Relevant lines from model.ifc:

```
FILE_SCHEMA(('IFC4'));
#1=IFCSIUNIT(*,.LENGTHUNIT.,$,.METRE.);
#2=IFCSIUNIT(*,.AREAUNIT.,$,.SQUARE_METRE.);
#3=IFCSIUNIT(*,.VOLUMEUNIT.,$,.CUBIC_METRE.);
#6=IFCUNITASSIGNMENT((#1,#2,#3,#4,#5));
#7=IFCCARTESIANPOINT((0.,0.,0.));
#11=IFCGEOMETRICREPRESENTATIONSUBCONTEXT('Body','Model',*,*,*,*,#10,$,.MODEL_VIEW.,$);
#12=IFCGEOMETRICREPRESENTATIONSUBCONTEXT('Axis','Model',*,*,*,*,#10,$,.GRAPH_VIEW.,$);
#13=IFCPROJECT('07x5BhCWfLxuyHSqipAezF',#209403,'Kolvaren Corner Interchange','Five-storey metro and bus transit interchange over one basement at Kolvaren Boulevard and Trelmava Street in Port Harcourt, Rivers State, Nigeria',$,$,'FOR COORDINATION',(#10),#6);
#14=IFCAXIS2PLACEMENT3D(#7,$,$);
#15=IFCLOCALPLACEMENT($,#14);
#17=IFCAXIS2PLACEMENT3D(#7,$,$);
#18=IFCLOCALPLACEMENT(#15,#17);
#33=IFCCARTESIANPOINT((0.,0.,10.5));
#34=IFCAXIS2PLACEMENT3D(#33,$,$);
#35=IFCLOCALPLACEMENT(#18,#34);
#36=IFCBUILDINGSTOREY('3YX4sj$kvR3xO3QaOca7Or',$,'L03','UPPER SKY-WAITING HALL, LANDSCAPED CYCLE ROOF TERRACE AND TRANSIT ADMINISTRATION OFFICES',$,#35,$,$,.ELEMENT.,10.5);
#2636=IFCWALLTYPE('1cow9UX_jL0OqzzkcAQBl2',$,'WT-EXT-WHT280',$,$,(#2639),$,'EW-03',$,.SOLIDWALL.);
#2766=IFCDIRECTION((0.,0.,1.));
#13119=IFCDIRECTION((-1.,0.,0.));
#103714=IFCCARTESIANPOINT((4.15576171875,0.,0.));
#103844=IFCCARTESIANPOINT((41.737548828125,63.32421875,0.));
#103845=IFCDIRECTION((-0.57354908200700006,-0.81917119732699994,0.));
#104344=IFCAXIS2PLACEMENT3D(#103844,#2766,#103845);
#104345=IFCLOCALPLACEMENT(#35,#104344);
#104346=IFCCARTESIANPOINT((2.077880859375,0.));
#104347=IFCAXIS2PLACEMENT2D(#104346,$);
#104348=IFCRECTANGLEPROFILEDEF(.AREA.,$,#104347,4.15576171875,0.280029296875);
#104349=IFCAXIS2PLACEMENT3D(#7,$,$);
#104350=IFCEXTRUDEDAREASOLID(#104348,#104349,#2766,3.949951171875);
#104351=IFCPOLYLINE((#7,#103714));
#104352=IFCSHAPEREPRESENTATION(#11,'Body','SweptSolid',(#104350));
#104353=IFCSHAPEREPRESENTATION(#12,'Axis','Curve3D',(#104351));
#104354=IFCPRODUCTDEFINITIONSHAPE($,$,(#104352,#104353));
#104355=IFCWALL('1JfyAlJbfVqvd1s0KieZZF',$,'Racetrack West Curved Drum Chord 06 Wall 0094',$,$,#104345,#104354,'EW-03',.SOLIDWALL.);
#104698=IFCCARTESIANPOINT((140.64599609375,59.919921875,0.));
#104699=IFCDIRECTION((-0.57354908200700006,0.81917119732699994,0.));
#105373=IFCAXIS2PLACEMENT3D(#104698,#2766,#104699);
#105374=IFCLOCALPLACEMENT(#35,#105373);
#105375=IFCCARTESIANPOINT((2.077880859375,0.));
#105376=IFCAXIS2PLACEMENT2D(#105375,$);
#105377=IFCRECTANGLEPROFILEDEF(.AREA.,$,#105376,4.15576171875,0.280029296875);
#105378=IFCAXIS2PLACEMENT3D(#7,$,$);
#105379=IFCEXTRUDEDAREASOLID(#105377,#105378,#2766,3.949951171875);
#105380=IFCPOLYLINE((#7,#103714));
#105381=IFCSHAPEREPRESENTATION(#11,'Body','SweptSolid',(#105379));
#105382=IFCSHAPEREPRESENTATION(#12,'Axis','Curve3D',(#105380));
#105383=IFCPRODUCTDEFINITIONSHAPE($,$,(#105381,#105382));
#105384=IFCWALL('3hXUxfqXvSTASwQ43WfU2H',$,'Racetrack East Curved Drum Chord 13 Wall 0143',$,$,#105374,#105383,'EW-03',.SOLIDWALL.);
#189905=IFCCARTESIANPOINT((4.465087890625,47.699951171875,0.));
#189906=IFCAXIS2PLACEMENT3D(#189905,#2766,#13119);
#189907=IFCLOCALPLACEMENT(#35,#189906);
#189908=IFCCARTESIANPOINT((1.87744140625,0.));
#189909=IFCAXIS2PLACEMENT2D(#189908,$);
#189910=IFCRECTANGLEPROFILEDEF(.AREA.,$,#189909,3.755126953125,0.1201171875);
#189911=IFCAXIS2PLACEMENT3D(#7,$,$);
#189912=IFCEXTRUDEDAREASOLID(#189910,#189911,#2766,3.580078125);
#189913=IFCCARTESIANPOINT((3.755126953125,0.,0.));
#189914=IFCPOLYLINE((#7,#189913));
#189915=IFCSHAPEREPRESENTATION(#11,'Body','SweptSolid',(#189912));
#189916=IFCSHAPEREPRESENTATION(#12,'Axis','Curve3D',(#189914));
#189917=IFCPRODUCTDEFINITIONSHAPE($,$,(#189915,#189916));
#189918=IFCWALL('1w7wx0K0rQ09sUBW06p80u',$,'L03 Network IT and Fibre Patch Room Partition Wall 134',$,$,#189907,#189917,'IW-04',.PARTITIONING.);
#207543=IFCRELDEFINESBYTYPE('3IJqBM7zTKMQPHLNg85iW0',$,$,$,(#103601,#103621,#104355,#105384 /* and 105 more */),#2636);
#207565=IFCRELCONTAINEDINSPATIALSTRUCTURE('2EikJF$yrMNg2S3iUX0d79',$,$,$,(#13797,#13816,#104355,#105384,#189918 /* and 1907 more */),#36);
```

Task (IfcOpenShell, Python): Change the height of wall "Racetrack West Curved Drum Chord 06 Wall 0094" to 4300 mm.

```python
import ifcopenshell
import ifcopenshell.geom
import ifcopenshell.util.representation
import ifcopenshell.util.shape

model = ifcopenshell.open("model.ifc")
settings = ifcopenshell.geom.settings()


def volume(element):
    """Net volume in cubic metres, openings subtracted."""
    shape = ifcopenshell.geom.create_shape(settings, element)
    return ifcopenshell.util.shape.get_volume(shape.geometry)


wall = model.by_guid("1JfyAlJbfVqvd1s0KieZZF")
before = volume(wall)

body = ifcopenshell.util.representation.get_representation(wall, "Model", "Body")
solid = body.Items[0]
old_height = solid.Depth
solid.Depth = 4.3
after = volume(wall)

print(f"height {old_height:g} -> {solid.Depth:g}, volume {before:.3f} -> {after:.3f} m3")

model.write("model_v2.ifc")
```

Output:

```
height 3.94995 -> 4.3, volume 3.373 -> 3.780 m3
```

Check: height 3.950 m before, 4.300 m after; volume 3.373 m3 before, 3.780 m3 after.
